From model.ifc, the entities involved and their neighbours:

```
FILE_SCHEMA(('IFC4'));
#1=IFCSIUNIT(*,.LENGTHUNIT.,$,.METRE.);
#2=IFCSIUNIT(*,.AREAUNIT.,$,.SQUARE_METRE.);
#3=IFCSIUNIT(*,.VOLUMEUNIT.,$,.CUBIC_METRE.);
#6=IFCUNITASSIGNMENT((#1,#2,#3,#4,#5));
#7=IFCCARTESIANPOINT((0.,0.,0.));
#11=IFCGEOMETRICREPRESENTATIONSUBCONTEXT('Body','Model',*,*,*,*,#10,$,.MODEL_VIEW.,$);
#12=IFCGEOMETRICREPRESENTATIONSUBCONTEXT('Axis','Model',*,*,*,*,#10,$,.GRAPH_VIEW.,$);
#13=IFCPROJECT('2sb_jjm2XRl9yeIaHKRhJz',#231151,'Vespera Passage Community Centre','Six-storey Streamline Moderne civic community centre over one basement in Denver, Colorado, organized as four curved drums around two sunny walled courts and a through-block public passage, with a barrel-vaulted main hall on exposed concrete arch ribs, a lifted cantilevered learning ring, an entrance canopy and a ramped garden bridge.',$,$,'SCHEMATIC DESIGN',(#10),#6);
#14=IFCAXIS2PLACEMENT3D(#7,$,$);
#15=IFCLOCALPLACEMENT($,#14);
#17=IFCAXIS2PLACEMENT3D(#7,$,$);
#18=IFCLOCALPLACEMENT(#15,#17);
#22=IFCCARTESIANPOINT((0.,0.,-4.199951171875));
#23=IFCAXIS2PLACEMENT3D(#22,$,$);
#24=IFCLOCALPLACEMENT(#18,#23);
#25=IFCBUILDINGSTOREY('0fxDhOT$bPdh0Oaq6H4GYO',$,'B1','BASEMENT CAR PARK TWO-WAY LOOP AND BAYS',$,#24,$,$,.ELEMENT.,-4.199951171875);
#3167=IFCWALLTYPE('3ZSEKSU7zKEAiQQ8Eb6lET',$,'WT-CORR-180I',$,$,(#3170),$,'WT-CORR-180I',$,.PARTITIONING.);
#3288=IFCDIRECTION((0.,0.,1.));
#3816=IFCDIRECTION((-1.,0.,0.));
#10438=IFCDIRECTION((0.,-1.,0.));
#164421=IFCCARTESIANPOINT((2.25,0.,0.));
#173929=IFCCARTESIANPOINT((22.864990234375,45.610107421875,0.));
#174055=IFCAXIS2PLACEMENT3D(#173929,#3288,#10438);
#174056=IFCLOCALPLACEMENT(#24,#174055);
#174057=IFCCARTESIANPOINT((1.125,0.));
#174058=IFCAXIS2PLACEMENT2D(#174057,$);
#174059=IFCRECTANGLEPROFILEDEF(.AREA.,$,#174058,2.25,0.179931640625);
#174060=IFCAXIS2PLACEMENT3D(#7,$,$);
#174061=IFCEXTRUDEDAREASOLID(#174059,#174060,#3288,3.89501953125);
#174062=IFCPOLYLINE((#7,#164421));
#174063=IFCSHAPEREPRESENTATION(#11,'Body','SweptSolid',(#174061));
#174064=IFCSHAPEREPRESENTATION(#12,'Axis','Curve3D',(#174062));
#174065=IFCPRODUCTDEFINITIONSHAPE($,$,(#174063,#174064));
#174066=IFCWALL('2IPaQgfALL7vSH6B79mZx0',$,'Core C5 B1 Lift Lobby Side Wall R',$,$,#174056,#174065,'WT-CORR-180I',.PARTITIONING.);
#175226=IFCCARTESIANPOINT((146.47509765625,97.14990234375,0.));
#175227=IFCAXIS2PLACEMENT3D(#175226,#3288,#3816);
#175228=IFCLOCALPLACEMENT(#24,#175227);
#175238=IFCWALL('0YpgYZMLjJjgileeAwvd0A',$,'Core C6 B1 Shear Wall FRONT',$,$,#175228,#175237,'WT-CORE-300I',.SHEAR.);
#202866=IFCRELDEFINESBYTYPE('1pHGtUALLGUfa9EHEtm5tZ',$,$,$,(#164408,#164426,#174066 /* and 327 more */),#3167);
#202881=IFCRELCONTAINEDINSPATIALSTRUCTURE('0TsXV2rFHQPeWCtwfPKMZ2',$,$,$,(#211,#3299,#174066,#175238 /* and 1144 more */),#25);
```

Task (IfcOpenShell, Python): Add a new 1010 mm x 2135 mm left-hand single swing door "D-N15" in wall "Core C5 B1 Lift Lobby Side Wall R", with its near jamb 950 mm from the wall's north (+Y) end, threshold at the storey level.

```python
import numpy as np
import ifcopenshell
import ifcopenshell.api.feature
import ifcopenshell.api.geometry
import ifcopenshell.api.root
import ifcopenshell.api.spatial
import ifcopenshell.geom
import ifcopenshell.util.element
import ifcopenshell.util.placement
import ifcopenshell.util.representation
import ifcopenshell.util.shape
import ifcopenshell.util.unit

model = ifcopenshell.open("model.ifc")
unit_scale = ifcopenshell.util.unit.calculate_unit_scale(model)
settings = ifcopenshell.geom.settings()


def volume(element):
    """Net volume in cubic metres, openings subtracted."""
    shape = ifcopenshell.geom.create_shape(settings, element)
    return ifcopenshell.util.shape.get_volume(shape.geometry)


wall = model.by_id(174066)
storey = ifcopenshell.util.element.get_container(wall, ifc_class="IfcBuildingStorey")
context = ifcopenshell.util.representation.get_context(model, "Model", "Body", "MODEL_VIEW")
before = volume(wall)

width, height, from_end, sill = 1.01, 2.135, 0.95, 0.0  # metres

# The wall runs along its own X axis, and the end named is its -X end.
wall_shape = ifcopenshell.geom.create_shape(settings, wall)
x, y, z = ifcopenshell.util.shape.get_vertices(wall_shape.geometry).T
start = x.min() + from_end
face, thickness = float(y.min()), float(y.max() - y.min())
wall_matrix = ifcopenshell.util.placement.get_local_placement(wall.ObjectPlacement)
level = ifcopenshell.util.placement.get_local_placement(storey.ObjectPlacement)[2, 3]


def in_wall(x, y):
    """Placement at x, y metres in the wall's axes, at sill height."""
    matrix = wall_matrix.copy()
    matrix[:, 3] = wall_matrix @ np.array([x / unit_scale, y / unit_scale, 0.0, 1.0])
    matrix[2, 3] = level + sill / unit_scale
    return matrix


# Opening: a box that overshoots both wall faces by 50 mm.
opening = ifcopenshell.api.root.create_entity(model, ifc_class="IfcOpeningElement", predefined_type="OPENING")
box = ifcopenshell.api.geometry.add_wall_representation(
    model, context=context, length=width, height=height, thickness=thickness + 0.1
)
ifcopenshell.api.geometry.assign_representation(model, product=opening, representation=box)
ifcopenshell.api.geometry.edit_object_placement(model, product=opening, matrix=in_wall(start, face - 0.05), is_si=False)
ifcopenshell.api.feature.add_feature(model, feature=opening, element=wall)

door = ifcopenshell.api.root.create_entity(model, ifc_class="IfcDoor", name="D-N15", predefined_type="DOOR")
door.OverallWidth, door.OverallHeight = width / unit_scale, height / unit_scale
door.OperationType = "SINGLE_SWING_LEFT"
body = ifcopenshell.api.geometry.add_door_representation(
    model,
    context=context,
    overall_width=door.OverallWidth,
    overall_height=door.OverallHeight,
    operation_type="SINGLE_SWING_LEFT",
    lining_properties={"LiningDepth": thickness / unit_scale, "ThresholdDepth": thickness / unit_scale},
)
ifcopenshell.api.geometry.assign_representation(model, product=door, representation=body)
ifcopenshell.api.spatial.assign_container(model, products=[door], relating_structure=storey)
ifcopenshell.api.feature.add_filling(model, opening=opening, element=door)

# The lining spans the wall, so the door starts at the wall face.
ifcopenshell.api.geometry.edit_object_placement(model, product=door, matrix=in_wall(start, face), is_si=False)

after = volume(wall)

print(f"wall volume {before:.3f} -> {after:.3f} m3")

model.write("model_v2.ifc")
```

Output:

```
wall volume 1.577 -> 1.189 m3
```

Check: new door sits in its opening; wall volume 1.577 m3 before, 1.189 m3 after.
